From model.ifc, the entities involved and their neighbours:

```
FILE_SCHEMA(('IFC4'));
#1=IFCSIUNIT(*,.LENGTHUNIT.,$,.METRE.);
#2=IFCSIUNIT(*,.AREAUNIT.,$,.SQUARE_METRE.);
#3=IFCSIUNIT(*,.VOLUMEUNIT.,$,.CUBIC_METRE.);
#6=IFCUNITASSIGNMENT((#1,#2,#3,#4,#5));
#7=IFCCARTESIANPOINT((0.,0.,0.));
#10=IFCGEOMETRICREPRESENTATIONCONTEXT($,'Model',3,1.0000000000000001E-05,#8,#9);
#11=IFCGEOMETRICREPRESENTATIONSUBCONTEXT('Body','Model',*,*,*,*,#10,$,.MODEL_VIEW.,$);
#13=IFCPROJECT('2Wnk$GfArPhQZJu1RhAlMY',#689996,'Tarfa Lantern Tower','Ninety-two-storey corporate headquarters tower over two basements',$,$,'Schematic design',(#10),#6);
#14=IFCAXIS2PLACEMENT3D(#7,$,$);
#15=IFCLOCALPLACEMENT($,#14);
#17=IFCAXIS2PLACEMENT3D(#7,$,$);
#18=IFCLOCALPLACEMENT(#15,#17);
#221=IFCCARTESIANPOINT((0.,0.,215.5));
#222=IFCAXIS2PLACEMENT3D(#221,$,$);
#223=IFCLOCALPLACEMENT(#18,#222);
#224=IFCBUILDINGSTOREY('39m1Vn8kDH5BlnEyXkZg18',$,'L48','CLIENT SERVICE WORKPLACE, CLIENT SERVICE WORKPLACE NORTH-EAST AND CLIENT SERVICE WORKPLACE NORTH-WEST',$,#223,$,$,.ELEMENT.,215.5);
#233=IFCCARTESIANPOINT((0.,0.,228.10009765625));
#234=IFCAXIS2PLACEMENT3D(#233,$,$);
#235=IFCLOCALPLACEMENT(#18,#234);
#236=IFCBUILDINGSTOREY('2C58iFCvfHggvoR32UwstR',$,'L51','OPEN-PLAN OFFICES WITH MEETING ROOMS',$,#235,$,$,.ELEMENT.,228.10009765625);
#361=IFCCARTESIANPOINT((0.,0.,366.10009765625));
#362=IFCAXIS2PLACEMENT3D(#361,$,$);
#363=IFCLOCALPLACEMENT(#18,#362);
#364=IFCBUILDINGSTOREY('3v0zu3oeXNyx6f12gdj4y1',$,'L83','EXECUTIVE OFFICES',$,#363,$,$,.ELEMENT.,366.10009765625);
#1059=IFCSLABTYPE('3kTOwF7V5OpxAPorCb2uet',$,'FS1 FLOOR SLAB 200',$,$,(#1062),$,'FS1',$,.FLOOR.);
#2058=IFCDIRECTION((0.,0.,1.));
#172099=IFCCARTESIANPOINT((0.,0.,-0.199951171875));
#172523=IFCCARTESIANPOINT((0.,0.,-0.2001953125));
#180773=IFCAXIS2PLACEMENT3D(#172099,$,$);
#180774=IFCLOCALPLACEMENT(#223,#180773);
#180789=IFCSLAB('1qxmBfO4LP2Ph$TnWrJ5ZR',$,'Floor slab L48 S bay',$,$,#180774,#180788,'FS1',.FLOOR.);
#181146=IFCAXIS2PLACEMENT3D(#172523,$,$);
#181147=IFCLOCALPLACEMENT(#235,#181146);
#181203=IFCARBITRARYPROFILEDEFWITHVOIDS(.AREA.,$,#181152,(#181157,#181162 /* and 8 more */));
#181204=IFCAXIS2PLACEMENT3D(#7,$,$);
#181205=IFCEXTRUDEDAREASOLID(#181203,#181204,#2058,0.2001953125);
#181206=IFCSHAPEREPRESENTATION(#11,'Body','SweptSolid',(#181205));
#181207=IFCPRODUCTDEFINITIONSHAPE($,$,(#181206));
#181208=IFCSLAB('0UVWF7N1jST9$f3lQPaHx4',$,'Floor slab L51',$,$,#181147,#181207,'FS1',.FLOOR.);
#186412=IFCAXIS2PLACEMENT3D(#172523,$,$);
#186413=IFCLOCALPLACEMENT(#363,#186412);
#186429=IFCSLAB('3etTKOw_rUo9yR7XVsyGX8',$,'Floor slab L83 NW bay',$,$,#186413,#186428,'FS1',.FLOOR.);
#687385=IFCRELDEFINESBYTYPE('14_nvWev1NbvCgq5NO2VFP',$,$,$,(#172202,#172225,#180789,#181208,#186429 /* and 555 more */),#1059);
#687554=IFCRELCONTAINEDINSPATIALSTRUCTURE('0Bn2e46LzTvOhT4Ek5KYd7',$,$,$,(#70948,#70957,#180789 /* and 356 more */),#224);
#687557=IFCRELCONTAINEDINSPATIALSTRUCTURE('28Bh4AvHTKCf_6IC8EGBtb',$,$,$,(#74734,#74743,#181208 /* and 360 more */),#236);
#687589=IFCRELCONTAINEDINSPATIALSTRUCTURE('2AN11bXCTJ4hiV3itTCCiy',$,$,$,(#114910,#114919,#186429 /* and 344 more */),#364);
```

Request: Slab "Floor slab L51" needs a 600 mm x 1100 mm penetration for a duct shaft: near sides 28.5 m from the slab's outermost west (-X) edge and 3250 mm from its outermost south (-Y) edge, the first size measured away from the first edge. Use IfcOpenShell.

```python
import numpy as np
import ifcopenshell
import ifcopenshell.api.feature
import ifcopenshell.api.geometry
import ifcopenshell.api.root
import ifcopenshell.geom
import ifcopenshell.util.placement
import ifcopenshell.util.representation
import ifcopenshell.util.shape
import ifcopenshell.util.unit

model = ifcopenshell.open("model.ifc")
unit_scale = ifcopenshell.util.unit.calculate_unit_scale(model)
settings = ifcopenshell.geom.settings()


def volume(element):
    """Net volume in cubic metres, openings subtracted."""
    shape = ifcopenshell.geom.create_shape(settings, element)
    return ifcopenshell.util.shape.get_volume(shape.geometry)


slab = model.by_guid("0UVWF7N1jST9$f3lQPaHx4")
before = volume(slab)

# Extent in the slab's own axes, in metres. The edges named are its -X and -Y sides.
slab_shape = ifcopenshell.geom.create_shape(settings, slab)
vertices = ifcopenshell.util.shape.get_vertices(slab_shape.geometry)
x_min, y_min, bottom = vertices.min(axis=0)
top = vertices[:, 2].max()

opening = ifcopenshell.api.root.create_entity(model, ifc_class="IfcOpeningElement", name="Duct shaft opening", predefined_type="OPENING")
context = ifcopenshell.util.representation.get_context(model, "Model", "Body", "MODEL_VIEW")
width, depth = 0.6, 1.1
outline = [(0.0, 0.0), (width, 0.0), (width, depth), (0.0, depth), (0.0, 0.0)]
# Overshoot both faces by 50 mm so the cut is clean.
shape = ifcopenshell.api.geometry.add_slab_representation(
    model, context=context, depth=top - bottom + 0.1, polyline=outline
)
ifcopenshell.api.geometry.assign_representation(model, product=opening, representation=shape)

matrix = ifcopenshell.util.placement.get_local_placement(slab.ObjectPlacement)
matrix[:, 3] = matrix @ np.append(np.array([x_min + 28.5, y_min + 3.25, bottom - 0.05]) / unit_scale, 1.0)
ifcopenshell.api.geometry.edit_object_placement(model, product=opening, matrix=matrix, is_si=False)
ifcopenshell.api.feature.add_feature(model, feature=opening, element=slab)

after = volume(slab)

print(f"slab volume {before:.3f} -> {after:.3f} m3")

model.write("model_edited.ifc")
```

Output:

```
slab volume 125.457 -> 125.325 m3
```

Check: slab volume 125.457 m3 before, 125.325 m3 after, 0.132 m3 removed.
